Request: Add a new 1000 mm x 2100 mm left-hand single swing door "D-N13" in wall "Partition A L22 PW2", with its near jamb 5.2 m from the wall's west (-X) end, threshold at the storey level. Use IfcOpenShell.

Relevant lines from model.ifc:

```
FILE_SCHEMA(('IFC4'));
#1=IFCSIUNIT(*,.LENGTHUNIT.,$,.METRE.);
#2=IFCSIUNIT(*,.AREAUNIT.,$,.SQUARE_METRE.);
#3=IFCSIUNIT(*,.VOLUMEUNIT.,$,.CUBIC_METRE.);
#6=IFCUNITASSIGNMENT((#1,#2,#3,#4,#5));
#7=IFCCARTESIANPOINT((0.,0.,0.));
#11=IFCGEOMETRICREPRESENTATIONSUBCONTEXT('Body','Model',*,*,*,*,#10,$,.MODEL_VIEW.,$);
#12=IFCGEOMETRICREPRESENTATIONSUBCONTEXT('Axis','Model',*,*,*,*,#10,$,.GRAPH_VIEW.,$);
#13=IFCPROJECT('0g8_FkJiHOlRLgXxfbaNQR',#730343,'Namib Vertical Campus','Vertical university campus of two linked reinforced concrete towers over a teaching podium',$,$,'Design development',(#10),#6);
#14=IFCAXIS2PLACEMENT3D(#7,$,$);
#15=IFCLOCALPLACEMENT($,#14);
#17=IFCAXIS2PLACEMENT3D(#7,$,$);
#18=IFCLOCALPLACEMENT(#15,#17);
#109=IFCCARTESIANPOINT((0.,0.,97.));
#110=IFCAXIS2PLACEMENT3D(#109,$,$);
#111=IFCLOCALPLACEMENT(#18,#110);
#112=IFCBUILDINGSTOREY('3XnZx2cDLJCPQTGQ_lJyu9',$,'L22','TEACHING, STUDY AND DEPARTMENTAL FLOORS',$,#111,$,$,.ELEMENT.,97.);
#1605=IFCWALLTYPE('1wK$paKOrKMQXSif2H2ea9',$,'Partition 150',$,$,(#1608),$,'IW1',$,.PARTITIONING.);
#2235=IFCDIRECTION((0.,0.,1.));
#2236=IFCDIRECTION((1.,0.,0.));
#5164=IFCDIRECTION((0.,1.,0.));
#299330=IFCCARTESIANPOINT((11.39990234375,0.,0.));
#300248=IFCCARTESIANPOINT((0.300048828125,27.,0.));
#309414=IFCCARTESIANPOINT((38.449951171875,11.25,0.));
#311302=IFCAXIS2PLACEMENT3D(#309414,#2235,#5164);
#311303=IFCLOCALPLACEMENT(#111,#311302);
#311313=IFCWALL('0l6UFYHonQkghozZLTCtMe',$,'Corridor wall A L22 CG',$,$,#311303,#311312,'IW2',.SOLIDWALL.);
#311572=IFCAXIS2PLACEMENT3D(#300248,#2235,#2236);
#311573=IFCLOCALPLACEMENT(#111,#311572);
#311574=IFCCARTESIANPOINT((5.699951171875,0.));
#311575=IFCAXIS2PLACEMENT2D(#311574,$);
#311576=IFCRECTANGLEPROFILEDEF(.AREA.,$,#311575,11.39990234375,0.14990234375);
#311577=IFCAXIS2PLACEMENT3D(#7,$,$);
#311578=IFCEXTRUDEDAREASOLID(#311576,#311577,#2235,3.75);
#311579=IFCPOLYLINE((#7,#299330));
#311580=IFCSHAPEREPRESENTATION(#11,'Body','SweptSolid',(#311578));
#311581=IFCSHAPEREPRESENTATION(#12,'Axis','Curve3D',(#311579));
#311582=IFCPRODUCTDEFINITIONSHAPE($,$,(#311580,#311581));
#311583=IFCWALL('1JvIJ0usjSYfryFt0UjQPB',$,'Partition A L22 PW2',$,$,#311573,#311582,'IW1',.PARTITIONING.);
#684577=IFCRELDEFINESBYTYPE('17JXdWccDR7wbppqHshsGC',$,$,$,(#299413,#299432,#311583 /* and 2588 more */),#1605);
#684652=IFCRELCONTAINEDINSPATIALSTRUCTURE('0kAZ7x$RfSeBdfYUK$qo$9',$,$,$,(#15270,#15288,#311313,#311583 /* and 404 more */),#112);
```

```python
import numpy as np
import ifcopenshell
import ifcopenshell.api.feature
import ifcopenshell.api.geometry
import ifcopenshell.api.root
import ifcopenshell.api.spatial
import ifcopenshell.geom
import ifcopenshell.util.element
import ifcopenshell.util.placement
import ifcopenshell.util.representation
import ifcopenshell.util.shape
import ifcopenshell.util.unit

model = ifcopenshell.open("model.ifc")
unit_scale = ifcopenshell.util.unit.calculate_unit_scale(model)
settings = ifcopenshell.geom.settings()


def volume(element):
    """Net volume in cubic metres, openings subtracted."""
    shape = ifcopenshell.geom.create_shape(settings, element)
    return ifcopenshell.util.shape.get_volume(shape.geometry)


wall = model.by_guid("1JvIJ0usjSYfryFt0UjQPB")
storey = ifcopenshell.util.element.get_container(wall, ifc_class="IfcBuildingStorey")
context = ifcopenshell.util.representation.get_context(model, "Model", "Body", "MODEL_VIEW")
before = volume(wall)

width, height, from_end, sill = 1, 2.1, 5.2, 0.0  # metres

# The wall runs along its own X axis, and the end named is its -X end.
wall_shape = ifcopenshell.geom.create_shape(settings, wall)
x, y, z = ifcopenshell.util.shape.get_vertices(wall_shape.geometry).T
start = x.min() + from_end
face, thickness = float(y.min()), float(y.max() - y.min())
wall_matrix = ifcopenshell.util.placement.get_local_placement(wall.ObjectPlacement)
level = ifcopenshell.util.placement.get_local_placement(storey.ObjectPlacement)[2, 3]


def in_wall(x, y):
    """Placement at x, y metres in the wall's axes, at sill height."""
    matrix = wall_matrix.copy()
    matrix[:, 3] = wall_matrix @ np.array([x / unit_scale, y / unit_scale, 0.0, 1.0])
    matrix[2, 3] = level + sill / unit_scale
    return matrix


# Opening: a box that overshoots both wall faces by 50 mm.
opening = ifcopenshell.api.root.create_entity(model, ifc_class="IfcOpeningElement", predefined_type="OPENING")
box = ifcopenshell.api.geometry.add_wall_representation(
    model, context=context, length=width, height=height, thickness=thickness + 0.1
)
ifcopenshell.api.geometry.assign_representation(model, product=opening, representation=box)
ifcopenshell.api.geometry.edit_object_placement(model, product=opening, matrix=in_wall(start, face - 0.05), is_si=False)
ifcopenshell.api.feature.add_feature(model, feature=opening, element=wall)

door = ifcopenshell.api.root.create_entity(model, ifc_class="IfcDoor", name="D-N13", predefined_type="DOOR")
door.OverallWidth, door.OverallHeight = width / unit_scale, height / unit_scale
door.OperationType = "SINGLE_SWING_LEFT"
body = ifcopenshell.api.geometry.add_door_representation(
    model,
    context=context,
    overall_width=door.OverallWidth,
    overall_height=door.OverallHeight,
    operation_type="SINGLE_SWING_LEFT",
    lining_properties={"LiningDepth": thickness / unit_scale, "ThresholdDepth": thickness / unit_scale},
)
ifcopenshell.api.geometry.assign_representation(model, product=door, representation=body)
ifcopenshell.api.spatial.assign_container(model, products=[door], relating_structure=storey)
ifcopenshell.api.feature.add_filling(model, opening=opening, element=door)

# The lining spans the wall, so the door starts at the wall face.
ifcopenshell.api.geometry.edit_object_placement(model, product=door, matrix=in_wall(start, face), is_si=False)

after = volume(wall)

print(f"wall volume {before:.3f} -> {after:.3f} m3")

model.write("model_updated.ifc")
```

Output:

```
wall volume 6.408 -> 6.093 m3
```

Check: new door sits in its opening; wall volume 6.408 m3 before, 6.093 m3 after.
